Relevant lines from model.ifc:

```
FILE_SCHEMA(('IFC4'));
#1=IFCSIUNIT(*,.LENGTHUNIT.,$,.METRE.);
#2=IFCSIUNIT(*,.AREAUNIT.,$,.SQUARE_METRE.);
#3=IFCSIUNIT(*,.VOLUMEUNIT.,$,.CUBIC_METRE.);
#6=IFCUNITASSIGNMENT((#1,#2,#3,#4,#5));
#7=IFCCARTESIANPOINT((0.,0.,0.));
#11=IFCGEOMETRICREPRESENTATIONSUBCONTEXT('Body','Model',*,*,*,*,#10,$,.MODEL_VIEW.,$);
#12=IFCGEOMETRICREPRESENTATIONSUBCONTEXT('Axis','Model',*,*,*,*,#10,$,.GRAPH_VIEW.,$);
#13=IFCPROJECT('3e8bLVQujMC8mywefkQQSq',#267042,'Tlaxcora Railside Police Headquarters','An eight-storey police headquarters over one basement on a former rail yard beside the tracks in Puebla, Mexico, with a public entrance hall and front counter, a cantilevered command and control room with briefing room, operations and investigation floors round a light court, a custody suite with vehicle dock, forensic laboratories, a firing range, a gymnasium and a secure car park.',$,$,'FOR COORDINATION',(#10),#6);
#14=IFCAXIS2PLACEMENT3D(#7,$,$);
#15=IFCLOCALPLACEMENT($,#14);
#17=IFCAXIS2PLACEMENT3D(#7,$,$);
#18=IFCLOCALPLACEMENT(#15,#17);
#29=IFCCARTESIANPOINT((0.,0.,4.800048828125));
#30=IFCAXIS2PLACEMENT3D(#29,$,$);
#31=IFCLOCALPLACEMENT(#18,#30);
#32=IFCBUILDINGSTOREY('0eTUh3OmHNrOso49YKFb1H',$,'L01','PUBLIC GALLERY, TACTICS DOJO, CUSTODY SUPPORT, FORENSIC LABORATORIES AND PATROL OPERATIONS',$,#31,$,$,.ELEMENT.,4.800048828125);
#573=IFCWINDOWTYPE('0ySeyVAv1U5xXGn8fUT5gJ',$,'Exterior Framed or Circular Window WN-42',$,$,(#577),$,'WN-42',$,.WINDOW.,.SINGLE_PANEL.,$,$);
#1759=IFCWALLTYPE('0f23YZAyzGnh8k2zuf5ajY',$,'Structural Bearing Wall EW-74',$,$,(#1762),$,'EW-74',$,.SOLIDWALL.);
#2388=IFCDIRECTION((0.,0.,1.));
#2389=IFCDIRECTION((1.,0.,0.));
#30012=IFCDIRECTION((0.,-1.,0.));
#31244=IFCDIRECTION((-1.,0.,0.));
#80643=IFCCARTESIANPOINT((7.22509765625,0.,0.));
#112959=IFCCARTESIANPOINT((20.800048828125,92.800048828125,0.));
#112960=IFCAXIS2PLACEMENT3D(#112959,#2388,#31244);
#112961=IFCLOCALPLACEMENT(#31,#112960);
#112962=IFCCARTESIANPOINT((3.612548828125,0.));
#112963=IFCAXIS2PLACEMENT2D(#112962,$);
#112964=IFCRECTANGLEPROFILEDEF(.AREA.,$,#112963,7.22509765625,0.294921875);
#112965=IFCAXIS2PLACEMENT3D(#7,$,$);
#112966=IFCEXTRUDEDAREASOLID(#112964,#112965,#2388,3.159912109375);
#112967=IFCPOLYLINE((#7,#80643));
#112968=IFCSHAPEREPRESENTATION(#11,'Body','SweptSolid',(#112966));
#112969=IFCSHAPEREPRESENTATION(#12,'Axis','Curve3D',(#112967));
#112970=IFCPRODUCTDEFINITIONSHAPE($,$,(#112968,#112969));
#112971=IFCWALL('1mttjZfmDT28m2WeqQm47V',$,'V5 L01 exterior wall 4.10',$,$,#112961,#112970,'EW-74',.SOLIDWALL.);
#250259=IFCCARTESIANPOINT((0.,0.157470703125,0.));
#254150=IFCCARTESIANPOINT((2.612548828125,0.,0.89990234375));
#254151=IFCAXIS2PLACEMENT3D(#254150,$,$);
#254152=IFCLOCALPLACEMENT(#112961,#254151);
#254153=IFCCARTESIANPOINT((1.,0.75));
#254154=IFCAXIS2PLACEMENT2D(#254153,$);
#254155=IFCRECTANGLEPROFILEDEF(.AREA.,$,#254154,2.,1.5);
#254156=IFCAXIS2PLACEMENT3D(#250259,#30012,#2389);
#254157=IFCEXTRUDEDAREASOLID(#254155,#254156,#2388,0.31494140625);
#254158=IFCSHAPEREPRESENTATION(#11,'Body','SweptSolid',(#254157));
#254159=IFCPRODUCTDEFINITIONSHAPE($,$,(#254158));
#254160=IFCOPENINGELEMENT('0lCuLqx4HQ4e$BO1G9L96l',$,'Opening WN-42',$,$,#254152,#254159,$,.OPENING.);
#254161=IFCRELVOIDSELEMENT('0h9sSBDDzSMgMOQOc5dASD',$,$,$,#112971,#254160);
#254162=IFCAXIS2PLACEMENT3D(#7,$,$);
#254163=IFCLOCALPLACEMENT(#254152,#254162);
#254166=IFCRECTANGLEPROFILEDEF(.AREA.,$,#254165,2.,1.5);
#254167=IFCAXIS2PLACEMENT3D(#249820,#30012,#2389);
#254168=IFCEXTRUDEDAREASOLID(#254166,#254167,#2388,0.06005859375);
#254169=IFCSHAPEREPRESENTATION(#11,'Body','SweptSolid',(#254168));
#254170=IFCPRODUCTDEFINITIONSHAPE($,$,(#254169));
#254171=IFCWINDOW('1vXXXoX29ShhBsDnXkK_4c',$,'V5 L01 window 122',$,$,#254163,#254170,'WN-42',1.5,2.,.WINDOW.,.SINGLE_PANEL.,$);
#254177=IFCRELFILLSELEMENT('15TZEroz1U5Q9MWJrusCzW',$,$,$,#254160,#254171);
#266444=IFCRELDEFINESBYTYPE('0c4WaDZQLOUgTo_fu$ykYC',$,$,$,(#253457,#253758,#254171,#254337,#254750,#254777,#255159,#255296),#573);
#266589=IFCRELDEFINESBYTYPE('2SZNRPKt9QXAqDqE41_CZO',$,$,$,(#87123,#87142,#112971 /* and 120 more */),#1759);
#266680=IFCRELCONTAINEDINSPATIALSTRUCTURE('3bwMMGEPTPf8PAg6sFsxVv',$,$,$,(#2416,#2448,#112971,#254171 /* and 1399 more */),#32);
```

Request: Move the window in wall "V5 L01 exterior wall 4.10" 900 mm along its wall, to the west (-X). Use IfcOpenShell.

```python
import ifcopenshell
import ifcopenshell.api.geometry
import ifcopenshell.util.placement
import ifcopenshell.util.unit

model = ifcopenshell.open("model.ifc")
unit_scale = ifcopenshell.util.unit.calculate_unit_scale(model)

window = model.by_guid("1vXXXoX29ShhBsDnXkK_4c")
opening = window.FillsVoids[0].RelatingOpeningElement
wall = opening.VoidsElements[0].RelatingBuildingElement

wall_matrix = ifcopenshell.util.placement.get_local_placement(wall.ObjectPlacement)
shift = wall_matrix[:3, 0] * 0.9 / unit_scale
before = ifcopenshell.util.placement.get_local_placement(window.ObjectPlacement)[:3, 3].copy()

# The window is placed relative to its opening, so it follows when the opening moves.
matrix = ifcopenshell.util.placement.get_local_placement(opening.ObjectPlacement)
matrix[:3, 3] += shift
ifcopenshell.api.geometry.edit_object_placement(
    model, product=opening, matrix=matrix, is_si=False, should_transform_children=True
)

after = ifcopenshell.util.placement.get_local_placement(window.ObjectPlacement)[:3, 3]
print("window moved by", (after - before).round(3) + 0.0)

model.write("model-out.ifc")
```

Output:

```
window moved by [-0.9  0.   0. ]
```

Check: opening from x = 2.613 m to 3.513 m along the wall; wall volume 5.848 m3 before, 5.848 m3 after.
